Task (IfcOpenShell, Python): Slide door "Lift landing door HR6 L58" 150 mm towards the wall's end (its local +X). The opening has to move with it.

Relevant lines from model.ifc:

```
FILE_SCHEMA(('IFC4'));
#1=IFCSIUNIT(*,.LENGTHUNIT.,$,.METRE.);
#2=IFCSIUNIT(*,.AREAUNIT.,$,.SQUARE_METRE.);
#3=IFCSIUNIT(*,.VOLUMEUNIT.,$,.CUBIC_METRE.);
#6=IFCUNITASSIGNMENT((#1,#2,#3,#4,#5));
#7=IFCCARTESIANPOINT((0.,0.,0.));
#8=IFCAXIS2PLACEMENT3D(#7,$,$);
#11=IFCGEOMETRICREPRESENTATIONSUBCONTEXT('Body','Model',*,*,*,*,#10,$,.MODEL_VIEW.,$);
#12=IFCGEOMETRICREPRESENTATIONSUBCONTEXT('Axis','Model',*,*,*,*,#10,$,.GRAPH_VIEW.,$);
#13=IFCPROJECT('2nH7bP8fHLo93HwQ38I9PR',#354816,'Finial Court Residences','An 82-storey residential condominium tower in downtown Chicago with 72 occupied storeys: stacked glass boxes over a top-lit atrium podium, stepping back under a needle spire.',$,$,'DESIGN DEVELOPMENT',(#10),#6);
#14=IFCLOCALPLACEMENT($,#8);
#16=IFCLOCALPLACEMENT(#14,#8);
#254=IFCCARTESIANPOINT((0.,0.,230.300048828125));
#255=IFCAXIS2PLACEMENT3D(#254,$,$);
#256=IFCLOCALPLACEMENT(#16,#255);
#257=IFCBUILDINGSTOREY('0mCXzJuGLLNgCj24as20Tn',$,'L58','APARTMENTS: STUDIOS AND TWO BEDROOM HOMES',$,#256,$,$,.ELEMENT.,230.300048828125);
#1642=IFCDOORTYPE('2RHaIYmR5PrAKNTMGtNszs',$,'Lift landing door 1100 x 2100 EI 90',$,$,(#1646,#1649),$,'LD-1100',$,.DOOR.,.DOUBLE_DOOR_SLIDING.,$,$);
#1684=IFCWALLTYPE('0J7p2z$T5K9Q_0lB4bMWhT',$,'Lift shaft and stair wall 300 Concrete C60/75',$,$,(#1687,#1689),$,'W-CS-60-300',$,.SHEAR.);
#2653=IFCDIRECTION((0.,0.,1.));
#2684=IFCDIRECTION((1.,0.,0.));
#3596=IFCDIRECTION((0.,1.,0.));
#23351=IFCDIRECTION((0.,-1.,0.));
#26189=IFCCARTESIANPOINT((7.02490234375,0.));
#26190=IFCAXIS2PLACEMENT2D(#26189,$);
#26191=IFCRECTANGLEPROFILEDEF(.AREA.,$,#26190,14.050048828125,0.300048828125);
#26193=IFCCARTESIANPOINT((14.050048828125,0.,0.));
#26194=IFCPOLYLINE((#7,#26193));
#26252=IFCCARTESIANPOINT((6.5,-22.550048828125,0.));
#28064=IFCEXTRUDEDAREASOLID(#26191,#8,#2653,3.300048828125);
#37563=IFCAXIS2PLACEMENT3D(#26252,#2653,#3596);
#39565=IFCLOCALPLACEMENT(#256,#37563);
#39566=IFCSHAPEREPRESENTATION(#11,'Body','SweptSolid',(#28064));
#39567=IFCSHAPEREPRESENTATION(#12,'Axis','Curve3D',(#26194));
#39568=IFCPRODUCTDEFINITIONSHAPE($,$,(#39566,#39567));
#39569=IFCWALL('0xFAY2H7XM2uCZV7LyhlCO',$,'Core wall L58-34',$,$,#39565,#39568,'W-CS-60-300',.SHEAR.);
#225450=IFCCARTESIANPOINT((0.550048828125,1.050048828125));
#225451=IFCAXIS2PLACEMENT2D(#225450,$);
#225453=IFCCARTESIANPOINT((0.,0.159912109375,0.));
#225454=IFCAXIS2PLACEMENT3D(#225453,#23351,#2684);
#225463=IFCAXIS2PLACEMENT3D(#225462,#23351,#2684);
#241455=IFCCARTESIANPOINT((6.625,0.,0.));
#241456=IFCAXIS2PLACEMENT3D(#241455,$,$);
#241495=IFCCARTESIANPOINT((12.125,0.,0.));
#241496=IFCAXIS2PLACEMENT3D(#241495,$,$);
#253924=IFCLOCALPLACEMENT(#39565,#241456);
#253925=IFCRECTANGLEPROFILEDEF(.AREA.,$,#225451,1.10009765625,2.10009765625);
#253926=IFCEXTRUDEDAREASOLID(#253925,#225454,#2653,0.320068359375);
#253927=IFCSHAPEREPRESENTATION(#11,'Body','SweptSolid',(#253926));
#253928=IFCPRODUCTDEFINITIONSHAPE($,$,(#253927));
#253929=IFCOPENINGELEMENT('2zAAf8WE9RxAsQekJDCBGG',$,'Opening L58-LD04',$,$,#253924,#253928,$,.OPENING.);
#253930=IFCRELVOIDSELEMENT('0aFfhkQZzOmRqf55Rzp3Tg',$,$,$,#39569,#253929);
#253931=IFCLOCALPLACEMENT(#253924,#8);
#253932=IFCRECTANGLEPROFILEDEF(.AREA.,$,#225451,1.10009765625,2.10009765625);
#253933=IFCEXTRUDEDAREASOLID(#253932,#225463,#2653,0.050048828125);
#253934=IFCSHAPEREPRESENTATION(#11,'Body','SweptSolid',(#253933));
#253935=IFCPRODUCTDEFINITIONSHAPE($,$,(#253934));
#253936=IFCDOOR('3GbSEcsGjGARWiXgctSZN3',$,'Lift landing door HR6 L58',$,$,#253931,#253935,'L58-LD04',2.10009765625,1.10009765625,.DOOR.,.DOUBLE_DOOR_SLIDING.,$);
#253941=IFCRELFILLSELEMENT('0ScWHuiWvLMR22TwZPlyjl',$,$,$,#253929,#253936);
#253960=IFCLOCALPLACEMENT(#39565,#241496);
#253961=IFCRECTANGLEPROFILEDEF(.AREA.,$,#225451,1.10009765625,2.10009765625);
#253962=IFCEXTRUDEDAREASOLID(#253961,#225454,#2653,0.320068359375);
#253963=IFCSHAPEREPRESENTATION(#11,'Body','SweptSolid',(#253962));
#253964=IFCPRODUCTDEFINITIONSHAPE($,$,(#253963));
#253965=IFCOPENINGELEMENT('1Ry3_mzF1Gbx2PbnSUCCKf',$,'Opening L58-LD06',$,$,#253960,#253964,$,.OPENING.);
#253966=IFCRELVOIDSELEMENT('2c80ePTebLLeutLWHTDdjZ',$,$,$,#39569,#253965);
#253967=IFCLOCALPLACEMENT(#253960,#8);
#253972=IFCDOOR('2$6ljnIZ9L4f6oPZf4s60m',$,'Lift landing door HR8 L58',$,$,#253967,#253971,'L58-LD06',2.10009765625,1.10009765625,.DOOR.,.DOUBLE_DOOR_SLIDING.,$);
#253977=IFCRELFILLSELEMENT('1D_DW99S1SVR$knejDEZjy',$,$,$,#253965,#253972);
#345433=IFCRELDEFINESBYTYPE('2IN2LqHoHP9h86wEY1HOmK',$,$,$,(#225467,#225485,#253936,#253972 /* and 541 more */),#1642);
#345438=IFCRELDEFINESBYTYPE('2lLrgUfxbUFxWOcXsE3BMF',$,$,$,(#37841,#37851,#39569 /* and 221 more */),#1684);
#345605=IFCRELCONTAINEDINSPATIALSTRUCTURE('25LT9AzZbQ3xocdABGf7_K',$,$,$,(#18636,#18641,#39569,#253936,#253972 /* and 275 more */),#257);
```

```python
import ifcopenshell
import ifcopenshell.api.geometry
import ifcopenshell.util.placement
import ifcopenshell.util.unit

model = ifcopenshell.open("model.ifc")
unit_scale = ifcopenshell.util.unit.calculate_unit_scale(model)

door = model.by_id(253936)
opening = door.FillsVoids[0].RelatingOpeningElement
wall = opening.VoidsElements[0].RelatingBuildingElement

wall_matrix = ifcopenshell.util.placement.get_local_placement(wall.ObjectPlacement)
shift = wall_matrix[:3, 0] * 0.15 / unit_scale
before = ifcopenshell.util.placement.get_local_placement(door.ObjectPlacement)[:3, 3].copy()

# The door is placed relative to its opening, so it follows when the opening moves.
matrix = ifcopenshell.util.placement.get_local_placement(opening.ObjectPlacement)
matrix[:3, 3] += shift
ifcopenshell.api.geometry.edit_object_placement(
    model, product=opening, matrix=matrix, is_si=False, should_transform_children=True
)

after = ifcopenshell.util.placement.get_local_placement(door.ObjectPlacement)[:3, 3]
print("door moved by", (after - before).round(3) + 0.0)

model.write("model_edited.ifc")
```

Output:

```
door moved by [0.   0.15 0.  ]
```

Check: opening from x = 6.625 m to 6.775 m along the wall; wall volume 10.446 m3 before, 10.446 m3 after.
